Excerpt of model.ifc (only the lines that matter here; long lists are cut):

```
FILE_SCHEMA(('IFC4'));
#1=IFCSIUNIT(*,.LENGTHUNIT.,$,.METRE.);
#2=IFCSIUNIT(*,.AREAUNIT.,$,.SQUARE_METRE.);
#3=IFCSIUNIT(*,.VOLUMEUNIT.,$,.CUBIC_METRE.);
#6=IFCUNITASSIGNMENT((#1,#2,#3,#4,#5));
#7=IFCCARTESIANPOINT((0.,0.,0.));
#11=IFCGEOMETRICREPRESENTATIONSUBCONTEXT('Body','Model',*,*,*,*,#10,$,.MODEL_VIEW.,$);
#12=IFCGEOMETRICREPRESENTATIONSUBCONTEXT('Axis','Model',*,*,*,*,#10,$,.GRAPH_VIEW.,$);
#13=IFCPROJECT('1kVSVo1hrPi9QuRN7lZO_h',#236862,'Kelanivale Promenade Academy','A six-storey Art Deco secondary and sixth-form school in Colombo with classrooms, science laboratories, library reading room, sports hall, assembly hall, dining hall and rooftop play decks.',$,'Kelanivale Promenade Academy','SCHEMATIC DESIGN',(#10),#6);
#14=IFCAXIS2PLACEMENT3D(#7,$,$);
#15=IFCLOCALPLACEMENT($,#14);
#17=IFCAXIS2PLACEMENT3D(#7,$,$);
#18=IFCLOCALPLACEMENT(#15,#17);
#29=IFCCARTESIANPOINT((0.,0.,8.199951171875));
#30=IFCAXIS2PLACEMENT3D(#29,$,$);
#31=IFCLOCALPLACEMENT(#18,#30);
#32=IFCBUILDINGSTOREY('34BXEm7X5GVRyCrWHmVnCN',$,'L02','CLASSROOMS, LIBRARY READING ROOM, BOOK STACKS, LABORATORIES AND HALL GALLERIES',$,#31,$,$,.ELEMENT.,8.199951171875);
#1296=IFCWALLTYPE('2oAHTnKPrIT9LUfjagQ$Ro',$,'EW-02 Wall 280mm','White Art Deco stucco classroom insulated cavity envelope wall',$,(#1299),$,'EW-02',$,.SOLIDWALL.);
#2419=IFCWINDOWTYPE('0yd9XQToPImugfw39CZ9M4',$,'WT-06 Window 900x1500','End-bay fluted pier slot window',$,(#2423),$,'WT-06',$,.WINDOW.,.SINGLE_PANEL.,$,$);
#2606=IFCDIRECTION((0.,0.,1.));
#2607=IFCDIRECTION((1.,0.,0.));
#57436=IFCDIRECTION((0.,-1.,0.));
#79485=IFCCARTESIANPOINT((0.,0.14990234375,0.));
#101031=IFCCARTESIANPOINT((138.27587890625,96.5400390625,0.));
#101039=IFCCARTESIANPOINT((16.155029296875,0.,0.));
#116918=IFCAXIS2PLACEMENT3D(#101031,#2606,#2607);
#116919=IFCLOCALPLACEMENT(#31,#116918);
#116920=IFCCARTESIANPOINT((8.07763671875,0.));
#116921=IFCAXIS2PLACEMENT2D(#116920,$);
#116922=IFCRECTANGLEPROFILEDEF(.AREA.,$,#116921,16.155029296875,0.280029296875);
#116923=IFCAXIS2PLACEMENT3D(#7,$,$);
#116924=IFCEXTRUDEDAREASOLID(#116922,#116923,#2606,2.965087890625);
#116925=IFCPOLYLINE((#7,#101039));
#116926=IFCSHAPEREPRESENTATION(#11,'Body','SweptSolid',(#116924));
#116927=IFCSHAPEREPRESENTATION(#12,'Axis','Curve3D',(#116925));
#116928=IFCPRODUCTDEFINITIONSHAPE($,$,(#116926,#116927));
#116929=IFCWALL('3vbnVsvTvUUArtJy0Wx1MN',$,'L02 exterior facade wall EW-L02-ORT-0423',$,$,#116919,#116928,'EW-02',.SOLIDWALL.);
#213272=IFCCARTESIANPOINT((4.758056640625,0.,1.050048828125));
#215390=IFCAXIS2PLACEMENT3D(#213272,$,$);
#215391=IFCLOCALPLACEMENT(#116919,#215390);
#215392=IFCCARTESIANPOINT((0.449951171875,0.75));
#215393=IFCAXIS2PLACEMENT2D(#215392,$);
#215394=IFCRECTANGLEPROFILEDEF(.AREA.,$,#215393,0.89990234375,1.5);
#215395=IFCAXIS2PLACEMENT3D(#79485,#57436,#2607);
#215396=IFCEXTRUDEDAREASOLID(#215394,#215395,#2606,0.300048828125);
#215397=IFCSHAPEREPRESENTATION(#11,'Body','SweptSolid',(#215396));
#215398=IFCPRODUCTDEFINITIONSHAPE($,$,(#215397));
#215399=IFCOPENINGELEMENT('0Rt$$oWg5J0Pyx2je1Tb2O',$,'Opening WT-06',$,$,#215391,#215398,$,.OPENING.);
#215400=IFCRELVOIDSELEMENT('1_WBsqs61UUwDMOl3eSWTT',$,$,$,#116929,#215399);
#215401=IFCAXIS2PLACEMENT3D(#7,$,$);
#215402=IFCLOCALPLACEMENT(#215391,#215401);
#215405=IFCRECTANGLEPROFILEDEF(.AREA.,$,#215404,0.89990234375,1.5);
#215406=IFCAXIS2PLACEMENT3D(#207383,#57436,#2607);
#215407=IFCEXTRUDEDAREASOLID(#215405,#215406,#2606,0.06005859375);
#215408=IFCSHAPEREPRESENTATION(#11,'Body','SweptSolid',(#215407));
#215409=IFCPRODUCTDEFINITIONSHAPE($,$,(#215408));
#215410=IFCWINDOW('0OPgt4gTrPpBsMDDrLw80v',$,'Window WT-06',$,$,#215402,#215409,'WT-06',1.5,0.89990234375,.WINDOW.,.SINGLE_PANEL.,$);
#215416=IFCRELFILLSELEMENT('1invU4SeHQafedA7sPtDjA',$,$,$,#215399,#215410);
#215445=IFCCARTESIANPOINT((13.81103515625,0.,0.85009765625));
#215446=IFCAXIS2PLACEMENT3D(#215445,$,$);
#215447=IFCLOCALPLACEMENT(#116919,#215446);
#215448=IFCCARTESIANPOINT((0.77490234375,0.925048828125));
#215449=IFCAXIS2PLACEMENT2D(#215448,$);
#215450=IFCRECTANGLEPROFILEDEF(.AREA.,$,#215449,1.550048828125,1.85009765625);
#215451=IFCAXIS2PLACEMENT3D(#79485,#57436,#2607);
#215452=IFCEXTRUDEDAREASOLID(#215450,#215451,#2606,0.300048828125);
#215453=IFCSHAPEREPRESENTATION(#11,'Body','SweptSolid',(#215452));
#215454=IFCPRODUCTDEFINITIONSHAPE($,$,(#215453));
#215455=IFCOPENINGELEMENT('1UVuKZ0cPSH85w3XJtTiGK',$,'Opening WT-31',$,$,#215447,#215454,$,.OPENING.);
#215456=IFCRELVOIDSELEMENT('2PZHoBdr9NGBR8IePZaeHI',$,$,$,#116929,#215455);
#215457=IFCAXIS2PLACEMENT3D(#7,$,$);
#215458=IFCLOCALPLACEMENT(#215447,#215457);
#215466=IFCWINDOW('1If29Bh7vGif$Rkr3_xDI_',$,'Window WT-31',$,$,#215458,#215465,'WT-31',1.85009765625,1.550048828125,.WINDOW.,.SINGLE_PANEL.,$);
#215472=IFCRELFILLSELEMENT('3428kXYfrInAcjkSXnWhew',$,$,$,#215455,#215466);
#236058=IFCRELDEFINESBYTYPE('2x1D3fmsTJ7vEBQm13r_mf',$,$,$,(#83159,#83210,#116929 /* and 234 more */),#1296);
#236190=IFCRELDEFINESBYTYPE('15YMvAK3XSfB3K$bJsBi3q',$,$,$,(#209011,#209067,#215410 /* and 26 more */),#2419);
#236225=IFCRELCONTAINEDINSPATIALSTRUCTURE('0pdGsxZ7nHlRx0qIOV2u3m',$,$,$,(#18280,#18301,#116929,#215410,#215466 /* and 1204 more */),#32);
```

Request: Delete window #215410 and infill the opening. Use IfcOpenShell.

```python
import ifcopenshell
import ifcopenshell.api.feature
import ifcopenshell.api.root
import ifcopenshell.geom
import ifcopenshell.util.shape

model = ifcopenshell.open("model.ifc")
settings = ifcopenshell.geom.settings()


def volume(element):
    """Net volume in cubic metres, openings subtracted."""
    shape = ifcopenshell.geom.create_shape(settings, element)
    return ifcopenshell.util.shape.get_volume(shape.geometry)


window = model.by_guid("0OPgt4gTrPpBsMDDrLw80v")
opening = window.FillsVoids[0].RelatingOpeningElement
wall = opening.VoidsElements[0].RelatingBuildingElement
before = volume(wall)

ifcopenshell.api.root.remove_product(model, product=window)
ifcopenshell.api.feature.remove_feature(model, feature=opening)

after = volume(wall)

print(f"wall volume {before:.3f} -> {after:.3f} m3")

model.write("model_updated.ifc")
```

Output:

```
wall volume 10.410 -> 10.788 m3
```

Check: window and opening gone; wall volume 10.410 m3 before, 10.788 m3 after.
